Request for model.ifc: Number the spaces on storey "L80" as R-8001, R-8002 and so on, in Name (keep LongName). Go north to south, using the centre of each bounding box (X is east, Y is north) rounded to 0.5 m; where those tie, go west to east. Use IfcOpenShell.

First a look at what the model holds.

```python
import ifcopenshell
import ifcopenshell.util.element
import ifcopenshell.util.placement

model = ifcopenshell.open("model.ifc")
print(model.schema)
storey = next(s for s in model.by_type("IfcBuildingStorey") if s.Name == "L80")
spaces = [e for e in ifcopenshell.util.element.get_decomposition(storey) if e.is_a("IfcSpace")]
for e in sorted(spaces, key=lambda e: e.id()):
    origin = ifcopenshell.util.placement.get_local_placement(e.ObjectPlacement)[:3, 3]
    print(e.id(), e.Name, e.LongName, origin.round(2) + 0.0, sep=" | ")
```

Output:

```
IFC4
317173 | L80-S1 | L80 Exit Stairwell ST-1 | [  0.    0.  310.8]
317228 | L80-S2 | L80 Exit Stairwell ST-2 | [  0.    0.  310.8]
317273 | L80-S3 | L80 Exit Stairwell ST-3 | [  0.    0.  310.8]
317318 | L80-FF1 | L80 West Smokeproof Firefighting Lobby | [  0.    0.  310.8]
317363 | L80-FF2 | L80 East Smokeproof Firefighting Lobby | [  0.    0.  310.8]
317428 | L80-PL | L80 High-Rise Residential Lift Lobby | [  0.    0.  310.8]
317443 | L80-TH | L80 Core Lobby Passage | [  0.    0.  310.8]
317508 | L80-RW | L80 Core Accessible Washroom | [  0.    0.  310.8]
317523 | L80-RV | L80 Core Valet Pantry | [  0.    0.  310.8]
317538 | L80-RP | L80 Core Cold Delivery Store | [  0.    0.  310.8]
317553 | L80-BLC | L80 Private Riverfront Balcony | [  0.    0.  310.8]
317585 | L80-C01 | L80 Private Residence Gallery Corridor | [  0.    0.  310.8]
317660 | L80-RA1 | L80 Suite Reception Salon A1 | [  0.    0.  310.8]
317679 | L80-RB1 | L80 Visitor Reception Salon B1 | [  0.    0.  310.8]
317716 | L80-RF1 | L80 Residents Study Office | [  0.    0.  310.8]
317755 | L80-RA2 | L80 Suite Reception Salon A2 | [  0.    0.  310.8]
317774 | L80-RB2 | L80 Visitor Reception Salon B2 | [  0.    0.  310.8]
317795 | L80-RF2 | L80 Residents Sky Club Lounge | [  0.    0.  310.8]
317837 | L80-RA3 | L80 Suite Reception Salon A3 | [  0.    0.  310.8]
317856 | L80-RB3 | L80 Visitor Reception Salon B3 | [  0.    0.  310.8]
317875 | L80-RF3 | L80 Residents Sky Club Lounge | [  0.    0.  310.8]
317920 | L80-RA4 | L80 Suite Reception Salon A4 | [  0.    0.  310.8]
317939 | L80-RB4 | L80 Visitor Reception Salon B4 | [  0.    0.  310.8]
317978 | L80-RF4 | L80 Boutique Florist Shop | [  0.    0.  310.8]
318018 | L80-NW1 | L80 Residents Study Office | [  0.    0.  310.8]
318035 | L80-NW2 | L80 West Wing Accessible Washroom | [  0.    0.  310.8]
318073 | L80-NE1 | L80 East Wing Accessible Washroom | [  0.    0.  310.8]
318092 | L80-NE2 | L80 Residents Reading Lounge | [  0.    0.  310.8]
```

```python
import ifcopenshell
import ifcopenshell.geom
import ifcopenshell.util.element
import ifcopenshell.util.shape

model = ifcopenshell.open("model.ifc")
settings = ifcopenshell.geom.settings()
settings.set("use-world-coords", True)


def centre(element):
    shape = ifcopenshell.geom.create_shape(settings, element)
    return ifcopenshell.util.shape.get_bbox_centroid(shape.geometry)


storey = next(s for s in model.by_type("IfcBuildingStorey") if s.Name == "L80")
spaces = [e for e in ifcopenshell.util.element.get_decomposition(storey) if e.is_a("IfcSpace")]

# Insertion points can sit at a corner or the storey origin, so sort by the geometry (in metres).
centres = {e: centre(e) for e in spaces}
spaces.sort(key=lambda e: (-round(centres[e][1] / 0.5), centres[e][0]))

for i, e in enumerate(spaces, start=1):
    number = f"R-80{i:02d}"
    e.Name = number
    print(e.id(), number)

model.write("model-out.ifc")
```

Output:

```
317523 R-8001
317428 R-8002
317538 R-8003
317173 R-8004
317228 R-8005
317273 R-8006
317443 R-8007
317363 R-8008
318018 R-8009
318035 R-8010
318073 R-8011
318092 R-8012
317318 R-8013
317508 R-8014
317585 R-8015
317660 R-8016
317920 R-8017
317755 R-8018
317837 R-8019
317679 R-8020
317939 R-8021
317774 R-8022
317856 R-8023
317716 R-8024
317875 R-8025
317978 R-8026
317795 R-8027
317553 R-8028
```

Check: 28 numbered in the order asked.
